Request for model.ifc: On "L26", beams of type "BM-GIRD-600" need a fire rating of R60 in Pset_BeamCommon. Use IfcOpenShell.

First a look at what the model holds.

```python
import ifcopenshell
import ifcopenshell.util.element

model = ifcopenshell.open("model.ifc")
print(model.schema)
storey = next(s for s in model.by_type("IfcBuildingStorey") if s.Name == "L26")
beams = [e for e in ifcopenshell.util.element.get_decomposition(storey) if e.is_a("IfcBeam")]
seen = {}
for e in beams:
    element_type = ifcopenshell.util.element.get_type(e)
    key = (element_type.Name if element_type != e and element_type else None, ifcopenshell.util.element.get_pset(e, "Pset_BeamCommon", "FireRating"))
    seen[key] = seen.get(key, 0) + 1
for (name, value), count in sorted(seen.items(), key=str):
    print(count, "x", name, "|", value)
```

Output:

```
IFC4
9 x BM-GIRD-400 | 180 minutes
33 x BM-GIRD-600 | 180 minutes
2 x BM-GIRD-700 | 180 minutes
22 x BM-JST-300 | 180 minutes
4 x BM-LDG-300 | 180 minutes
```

```python
import ifcopenshell
import ifcopenshell.api.pset
import ifcopenshell.util.element

model = ifcopenshell.open("model.ifc")

storey = next(s for s in model.by_type("IfcBuildingStorey") if s.Name == "L26")
beams = [e for e in ifcopenshell.util.element.get_decomposition(storey) if e.is_a("IfcBeam")]

count = 0
for e in beams:
    element_type = ifcopenshell.util.element.get_type(e)
    if element_type in (None, e) or element_type.Name != "BM-GIRD-600":
        continue
    found = ifcopenshell.util.element.get_pset(e, "Pset_BeamCommon", should_inherit=False)
    if found:
        pset = model.by_id(found["id"])
        if len(ifcopenshell.util.element.get_elements_by_pset(pset)) > 1:
            pset = ifcopenshell.api.pset.unshare_pset(model, products=[e], pset=pset)[0]
    else:
        pset = ifcopenshell.api.pset.add_pset(model, product=e, name="Pset_BeamCommon")
    ifcopenshell.api.pset.edit_pset(model, pset=pset, properties={"FireRating": "R60"})
    count += 1

print(count, "beams updated")

model.write("model_rev.ifc")
```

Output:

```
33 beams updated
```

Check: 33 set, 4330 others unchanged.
